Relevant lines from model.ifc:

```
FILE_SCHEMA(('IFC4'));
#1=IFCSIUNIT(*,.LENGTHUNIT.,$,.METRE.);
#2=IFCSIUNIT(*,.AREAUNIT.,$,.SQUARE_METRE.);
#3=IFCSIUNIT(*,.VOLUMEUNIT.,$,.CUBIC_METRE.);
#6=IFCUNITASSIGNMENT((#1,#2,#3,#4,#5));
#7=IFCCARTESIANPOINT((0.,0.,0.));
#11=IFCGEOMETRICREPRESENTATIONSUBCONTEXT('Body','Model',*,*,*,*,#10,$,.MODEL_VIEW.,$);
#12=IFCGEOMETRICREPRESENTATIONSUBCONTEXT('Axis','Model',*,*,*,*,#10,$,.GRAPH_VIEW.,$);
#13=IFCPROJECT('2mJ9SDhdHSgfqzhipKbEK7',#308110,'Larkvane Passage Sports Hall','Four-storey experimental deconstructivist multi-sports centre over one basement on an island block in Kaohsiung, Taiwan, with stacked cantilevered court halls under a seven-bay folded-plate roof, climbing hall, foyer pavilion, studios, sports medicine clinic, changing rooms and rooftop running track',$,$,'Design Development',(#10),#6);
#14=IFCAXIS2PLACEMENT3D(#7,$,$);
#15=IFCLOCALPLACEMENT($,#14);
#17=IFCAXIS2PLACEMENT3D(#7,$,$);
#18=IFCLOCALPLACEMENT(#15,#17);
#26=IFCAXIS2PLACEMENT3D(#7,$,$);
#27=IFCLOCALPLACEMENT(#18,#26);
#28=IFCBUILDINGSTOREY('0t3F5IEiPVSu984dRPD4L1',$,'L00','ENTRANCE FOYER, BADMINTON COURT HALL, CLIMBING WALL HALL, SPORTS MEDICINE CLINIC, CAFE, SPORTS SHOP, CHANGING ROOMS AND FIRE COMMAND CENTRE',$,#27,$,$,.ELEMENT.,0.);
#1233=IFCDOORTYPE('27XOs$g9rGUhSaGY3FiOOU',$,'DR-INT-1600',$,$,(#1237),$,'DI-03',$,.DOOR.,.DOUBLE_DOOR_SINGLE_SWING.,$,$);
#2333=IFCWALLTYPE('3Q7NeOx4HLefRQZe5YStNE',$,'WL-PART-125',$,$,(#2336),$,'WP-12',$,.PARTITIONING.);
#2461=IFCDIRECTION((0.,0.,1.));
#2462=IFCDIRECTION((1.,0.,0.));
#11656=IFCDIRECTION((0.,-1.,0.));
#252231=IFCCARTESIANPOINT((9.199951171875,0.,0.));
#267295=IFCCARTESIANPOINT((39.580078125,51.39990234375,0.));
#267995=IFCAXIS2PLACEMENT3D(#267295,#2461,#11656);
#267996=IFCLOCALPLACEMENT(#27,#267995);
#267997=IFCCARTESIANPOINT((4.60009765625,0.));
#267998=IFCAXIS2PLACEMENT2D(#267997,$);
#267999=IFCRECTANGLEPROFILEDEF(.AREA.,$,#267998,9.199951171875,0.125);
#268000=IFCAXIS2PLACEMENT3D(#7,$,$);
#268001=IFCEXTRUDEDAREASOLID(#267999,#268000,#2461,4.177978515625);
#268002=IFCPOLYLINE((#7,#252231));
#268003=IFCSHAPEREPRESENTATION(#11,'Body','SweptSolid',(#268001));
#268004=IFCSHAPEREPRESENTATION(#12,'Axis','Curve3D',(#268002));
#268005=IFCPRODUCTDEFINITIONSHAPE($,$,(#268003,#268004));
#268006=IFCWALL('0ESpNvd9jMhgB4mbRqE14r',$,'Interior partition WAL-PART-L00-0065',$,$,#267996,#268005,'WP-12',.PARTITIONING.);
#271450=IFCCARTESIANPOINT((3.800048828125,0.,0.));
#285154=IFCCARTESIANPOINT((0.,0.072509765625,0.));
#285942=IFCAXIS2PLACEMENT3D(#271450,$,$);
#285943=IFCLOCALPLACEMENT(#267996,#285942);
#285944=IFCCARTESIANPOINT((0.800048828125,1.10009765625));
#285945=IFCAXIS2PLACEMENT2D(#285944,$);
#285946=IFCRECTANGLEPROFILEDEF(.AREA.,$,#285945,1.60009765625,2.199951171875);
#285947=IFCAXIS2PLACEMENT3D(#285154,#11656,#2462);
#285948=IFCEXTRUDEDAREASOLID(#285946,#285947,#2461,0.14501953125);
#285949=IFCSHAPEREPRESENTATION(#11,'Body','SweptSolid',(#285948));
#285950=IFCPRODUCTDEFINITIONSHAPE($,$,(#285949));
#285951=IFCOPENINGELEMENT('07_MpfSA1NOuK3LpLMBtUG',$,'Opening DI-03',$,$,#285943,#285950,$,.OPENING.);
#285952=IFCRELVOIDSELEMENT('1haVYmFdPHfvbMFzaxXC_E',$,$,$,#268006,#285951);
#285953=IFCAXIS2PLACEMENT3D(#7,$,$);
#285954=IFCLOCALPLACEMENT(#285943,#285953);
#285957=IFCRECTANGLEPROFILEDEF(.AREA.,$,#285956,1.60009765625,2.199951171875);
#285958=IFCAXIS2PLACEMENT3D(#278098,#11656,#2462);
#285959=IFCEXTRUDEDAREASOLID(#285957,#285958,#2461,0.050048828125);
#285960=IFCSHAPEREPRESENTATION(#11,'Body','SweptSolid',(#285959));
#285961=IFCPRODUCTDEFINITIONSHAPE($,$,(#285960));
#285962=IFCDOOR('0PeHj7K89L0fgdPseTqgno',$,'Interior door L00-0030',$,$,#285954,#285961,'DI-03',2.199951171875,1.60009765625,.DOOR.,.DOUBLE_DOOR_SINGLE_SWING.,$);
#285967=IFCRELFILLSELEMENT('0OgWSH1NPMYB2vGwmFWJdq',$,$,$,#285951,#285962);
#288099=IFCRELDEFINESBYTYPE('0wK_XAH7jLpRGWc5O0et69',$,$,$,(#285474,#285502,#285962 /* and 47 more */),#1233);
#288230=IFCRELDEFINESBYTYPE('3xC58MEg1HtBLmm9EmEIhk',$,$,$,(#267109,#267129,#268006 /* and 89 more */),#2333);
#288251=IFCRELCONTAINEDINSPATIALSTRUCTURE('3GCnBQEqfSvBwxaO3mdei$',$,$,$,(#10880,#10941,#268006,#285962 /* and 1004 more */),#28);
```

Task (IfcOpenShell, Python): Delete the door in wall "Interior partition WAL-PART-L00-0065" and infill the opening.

```python
import ifcopenshell
import ifcopenshell.api.feature
import ifcopenshell.api.root
import ifcopenshell.geom
import ifcopenshell.util.shape

model = ifcopenshell.open("model.ifc")
settings = ifcopenshell.geom.settings()


def volume(element):
    """Net volume in cubic metres, openings subtracted."""
    shape = ifcopenshell.geom.create_shape(settings, element)
    return ifcopenshell.util.shape.get_volume(shape.geometry)


door = model.by_guid("0PeHj7K89L0fgdPseTqgno")
opening = door.FillsVoids[0].RelatingOpeningElement
wall = opening.VoidsElements[0].RelatingBuildingElement
before = volume(wall)

ifcopenshell.api.root.remove_product(model, product=door)
ifcopenshell.api.feature.remove_feature(model, feature=opening)

after = volume(wall)

print(f"wall volume {before:.3f} -> {after:.3f} m3")

model.write("model_updated.ifc")
```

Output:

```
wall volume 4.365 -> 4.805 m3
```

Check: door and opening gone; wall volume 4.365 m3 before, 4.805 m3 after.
